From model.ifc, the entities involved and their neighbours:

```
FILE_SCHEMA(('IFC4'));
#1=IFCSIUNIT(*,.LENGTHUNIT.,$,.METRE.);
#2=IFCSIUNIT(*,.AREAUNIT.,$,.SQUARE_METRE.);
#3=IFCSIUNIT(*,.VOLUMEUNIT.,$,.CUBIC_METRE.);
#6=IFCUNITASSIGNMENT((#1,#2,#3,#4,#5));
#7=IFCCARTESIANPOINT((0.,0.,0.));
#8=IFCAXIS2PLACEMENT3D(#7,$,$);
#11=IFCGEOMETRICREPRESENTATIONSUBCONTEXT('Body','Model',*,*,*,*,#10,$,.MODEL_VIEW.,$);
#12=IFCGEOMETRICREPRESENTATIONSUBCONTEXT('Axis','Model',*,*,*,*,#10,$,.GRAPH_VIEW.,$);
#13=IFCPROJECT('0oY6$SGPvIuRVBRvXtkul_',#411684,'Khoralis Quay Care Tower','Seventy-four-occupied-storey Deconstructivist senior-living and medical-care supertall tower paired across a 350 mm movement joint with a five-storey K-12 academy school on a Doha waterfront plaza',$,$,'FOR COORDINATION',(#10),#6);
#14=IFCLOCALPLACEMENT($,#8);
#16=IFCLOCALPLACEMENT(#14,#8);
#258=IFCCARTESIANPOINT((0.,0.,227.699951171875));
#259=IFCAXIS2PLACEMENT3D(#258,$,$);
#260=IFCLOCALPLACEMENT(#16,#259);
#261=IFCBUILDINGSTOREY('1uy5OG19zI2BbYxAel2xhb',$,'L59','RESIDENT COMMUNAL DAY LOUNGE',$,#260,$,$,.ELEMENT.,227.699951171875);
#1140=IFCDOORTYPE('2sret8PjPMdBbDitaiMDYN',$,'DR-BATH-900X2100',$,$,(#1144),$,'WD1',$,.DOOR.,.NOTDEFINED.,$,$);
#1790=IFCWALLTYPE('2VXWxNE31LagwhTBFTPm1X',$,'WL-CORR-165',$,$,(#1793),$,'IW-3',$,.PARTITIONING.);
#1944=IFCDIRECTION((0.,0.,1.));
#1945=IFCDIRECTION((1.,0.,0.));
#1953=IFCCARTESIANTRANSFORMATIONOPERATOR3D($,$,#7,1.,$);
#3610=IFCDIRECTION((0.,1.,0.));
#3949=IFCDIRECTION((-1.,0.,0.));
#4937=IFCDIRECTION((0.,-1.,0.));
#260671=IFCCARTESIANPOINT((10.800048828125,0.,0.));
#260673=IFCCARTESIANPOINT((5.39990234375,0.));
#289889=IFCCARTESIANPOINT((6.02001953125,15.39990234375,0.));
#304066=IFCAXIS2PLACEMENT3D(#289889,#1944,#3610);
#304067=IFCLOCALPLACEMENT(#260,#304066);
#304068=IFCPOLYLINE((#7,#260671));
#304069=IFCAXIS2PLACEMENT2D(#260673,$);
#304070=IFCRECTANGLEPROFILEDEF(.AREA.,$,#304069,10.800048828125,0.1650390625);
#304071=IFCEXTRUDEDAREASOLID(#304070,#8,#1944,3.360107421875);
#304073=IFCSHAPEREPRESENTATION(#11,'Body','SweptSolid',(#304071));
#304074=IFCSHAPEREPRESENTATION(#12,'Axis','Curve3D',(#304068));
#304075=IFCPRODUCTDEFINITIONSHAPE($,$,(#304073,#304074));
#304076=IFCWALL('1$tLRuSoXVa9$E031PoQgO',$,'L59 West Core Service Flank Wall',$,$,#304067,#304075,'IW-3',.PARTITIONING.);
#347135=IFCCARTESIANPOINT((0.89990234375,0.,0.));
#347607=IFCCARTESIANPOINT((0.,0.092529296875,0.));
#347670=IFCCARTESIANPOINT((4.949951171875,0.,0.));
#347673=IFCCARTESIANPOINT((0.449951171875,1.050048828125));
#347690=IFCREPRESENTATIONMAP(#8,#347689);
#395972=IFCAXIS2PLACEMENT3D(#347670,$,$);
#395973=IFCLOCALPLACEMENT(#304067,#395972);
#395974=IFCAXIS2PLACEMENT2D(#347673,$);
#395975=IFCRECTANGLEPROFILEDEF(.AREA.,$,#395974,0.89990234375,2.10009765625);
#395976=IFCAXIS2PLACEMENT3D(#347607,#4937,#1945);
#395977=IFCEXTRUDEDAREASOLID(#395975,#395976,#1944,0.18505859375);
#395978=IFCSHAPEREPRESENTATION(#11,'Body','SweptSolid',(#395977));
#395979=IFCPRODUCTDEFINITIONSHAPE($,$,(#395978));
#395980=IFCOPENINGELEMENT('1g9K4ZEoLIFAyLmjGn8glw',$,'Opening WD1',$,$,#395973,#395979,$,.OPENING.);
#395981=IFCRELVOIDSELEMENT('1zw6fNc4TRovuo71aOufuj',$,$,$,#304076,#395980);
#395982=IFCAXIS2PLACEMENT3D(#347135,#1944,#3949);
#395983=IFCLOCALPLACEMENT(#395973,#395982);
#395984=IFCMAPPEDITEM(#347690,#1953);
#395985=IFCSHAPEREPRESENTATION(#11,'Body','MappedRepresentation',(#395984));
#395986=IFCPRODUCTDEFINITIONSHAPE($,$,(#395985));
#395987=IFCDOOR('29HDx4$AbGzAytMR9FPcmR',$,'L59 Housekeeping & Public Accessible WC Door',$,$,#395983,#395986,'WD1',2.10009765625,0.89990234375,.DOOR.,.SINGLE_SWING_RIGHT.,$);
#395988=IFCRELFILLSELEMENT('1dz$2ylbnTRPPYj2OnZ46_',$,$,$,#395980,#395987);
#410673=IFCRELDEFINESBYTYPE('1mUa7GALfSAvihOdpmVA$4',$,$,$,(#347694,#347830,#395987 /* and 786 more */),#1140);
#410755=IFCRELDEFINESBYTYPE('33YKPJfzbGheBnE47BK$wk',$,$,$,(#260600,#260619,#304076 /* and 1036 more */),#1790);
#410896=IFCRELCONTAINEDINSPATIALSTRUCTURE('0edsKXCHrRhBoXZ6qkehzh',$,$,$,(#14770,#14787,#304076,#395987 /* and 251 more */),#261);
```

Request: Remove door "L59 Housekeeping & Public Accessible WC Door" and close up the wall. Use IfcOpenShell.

```python
import ifcopenshell
import ifcopenshell.api.feature
import ifcopenshell.api.root
import ifcopenshell.geom
import ifcopenshell.util.shape

model = ifcopenshell.open("model.ifc")
settings = ifcopenshell.geom.settings()


def volume(element):
    """Net volume in cubic metres, openings subtracted."""
    shape = ifcopenshell.geom.create_shape(settings, element)
    return ifcopenshell.util.shape.get_volume(shape.geometry)


door = model.by_guid("29HDx4$AbGzAytMR9FPcmR")
opening = door.FillsVoids[0].RelatingOpeningElement
wall = opening.VoidsElements[0].RelatingBuildingElement
before = volume(wall)

ifcopenshell.api.root.remove_product(model, product=door)
ifcopenshell.api.feature.remove_feature(model, feature=opening)

after = volume(wall)

print(f"wall volume {before:.3f} -> {after:.3f} m3")

model.write("model_rev.ifc")
```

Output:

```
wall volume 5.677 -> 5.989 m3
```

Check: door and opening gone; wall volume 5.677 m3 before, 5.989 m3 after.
